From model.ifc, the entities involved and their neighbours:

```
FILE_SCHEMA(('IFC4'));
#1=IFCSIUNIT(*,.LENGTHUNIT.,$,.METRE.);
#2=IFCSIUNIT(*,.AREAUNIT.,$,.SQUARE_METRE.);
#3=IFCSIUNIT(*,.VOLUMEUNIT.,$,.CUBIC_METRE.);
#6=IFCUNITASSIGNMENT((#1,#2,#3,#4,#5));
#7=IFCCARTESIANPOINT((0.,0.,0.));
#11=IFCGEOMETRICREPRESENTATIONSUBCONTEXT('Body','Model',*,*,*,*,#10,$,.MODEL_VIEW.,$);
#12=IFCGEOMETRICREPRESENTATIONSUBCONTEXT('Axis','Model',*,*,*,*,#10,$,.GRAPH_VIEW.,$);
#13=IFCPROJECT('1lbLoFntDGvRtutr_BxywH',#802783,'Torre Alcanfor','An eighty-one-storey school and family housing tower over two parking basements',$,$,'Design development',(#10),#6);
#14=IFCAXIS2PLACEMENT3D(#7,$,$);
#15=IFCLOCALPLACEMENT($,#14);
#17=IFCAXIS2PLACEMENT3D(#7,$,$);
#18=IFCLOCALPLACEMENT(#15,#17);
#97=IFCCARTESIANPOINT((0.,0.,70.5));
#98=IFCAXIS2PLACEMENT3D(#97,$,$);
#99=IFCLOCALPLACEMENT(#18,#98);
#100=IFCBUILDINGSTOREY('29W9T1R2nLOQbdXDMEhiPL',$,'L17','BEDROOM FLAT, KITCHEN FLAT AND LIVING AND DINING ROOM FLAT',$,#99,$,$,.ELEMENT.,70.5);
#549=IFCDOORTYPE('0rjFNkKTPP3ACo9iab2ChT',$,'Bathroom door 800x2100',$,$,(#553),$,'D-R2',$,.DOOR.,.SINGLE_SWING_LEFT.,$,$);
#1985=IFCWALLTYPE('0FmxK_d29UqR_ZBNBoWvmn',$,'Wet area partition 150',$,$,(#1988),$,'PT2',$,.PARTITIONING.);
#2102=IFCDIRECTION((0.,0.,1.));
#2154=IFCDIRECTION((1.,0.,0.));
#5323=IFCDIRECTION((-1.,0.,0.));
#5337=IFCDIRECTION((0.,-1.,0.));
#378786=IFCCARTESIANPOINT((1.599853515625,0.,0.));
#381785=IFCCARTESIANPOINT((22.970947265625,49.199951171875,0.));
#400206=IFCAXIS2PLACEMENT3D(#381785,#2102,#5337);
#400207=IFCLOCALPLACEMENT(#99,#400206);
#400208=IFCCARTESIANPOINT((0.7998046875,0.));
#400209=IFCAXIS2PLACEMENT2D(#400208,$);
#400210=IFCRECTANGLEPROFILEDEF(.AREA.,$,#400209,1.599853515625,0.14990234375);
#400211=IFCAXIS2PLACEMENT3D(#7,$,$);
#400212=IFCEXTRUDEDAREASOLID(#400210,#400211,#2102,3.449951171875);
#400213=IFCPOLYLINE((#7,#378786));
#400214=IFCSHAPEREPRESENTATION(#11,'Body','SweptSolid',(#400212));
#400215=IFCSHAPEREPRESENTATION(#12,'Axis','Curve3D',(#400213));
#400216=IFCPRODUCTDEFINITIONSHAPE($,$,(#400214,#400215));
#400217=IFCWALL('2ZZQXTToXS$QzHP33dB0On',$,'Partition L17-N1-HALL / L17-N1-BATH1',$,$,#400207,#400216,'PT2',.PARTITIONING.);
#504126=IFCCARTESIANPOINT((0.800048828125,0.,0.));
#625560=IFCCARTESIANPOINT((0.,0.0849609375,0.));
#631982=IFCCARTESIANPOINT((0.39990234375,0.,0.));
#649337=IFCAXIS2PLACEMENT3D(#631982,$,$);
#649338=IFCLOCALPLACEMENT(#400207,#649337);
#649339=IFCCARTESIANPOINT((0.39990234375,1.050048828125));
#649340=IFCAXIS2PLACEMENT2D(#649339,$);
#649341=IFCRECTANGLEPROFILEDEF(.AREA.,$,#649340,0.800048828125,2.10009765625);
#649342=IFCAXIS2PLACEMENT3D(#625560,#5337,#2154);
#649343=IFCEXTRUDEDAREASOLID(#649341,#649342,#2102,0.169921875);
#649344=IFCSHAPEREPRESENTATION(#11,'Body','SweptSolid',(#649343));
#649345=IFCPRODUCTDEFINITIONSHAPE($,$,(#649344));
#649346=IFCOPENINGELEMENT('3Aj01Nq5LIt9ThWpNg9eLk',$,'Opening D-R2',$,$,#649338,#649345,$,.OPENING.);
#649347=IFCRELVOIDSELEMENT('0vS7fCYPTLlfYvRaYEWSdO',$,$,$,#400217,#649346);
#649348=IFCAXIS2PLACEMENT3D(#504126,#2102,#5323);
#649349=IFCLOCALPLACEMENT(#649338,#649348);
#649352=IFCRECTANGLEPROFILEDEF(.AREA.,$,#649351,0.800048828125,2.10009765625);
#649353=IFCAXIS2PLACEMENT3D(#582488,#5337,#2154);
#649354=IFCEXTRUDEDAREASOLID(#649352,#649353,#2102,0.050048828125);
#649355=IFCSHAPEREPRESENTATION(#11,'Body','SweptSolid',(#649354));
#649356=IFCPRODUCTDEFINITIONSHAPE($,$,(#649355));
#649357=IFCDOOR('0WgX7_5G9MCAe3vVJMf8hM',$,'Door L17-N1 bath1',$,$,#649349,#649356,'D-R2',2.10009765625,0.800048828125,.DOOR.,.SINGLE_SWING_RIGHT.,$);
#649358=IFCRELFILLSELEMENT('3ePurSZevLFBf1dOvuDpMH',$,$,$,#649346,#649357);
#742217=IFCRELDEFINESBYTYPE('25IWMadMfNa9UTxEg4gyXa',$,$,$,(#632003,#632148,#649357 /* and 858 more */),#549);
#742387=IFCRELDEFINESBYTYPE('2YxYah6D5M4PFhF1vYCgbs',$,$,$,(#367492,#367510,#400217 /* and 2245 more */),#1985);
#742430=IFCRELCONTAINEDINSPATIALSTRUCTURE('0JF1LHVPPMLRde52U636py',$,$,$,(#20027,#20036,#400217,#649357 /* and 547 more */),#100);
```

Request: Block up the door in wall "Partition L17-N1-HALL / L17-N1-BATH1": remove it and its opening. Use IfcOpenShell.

```python
import ifcopenshell
import ifcopenshell.api.feature
import ifcopenshell.api.root
import ifcopenshell.geom
import ifcopenshell.util.shape

model = ifcopenshell.open("model.ifc")
settings = ifcopenshell.geom.settings()


def volume(element):
    """Net volume in cubic metres, openings subtracted."""
    shape = ifcopenshell.geom.create_shape(settings, element)
    return ifcopenshell.util.shape.get_volume(shape.geometry)


door = model.by_id(649357)
opening = door.FillsVoids[0].RelatingOpeningElement
wall = opening.VoidsElements[0].RelatingBuildingElement
before = volume(wall)

ifcopenshell.api.root.remove_product(model, product=door)
ifcopenshell.api.feature.remove_feature(model, feature=opening)

after = volume(wall)

print(f"wall volume {before:.3f} -> {after:.3f} m3")

model.write("model_rev.ifc")
```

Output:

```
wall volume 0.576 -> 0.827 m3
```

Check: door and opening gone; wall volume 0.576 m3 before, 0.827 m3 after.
